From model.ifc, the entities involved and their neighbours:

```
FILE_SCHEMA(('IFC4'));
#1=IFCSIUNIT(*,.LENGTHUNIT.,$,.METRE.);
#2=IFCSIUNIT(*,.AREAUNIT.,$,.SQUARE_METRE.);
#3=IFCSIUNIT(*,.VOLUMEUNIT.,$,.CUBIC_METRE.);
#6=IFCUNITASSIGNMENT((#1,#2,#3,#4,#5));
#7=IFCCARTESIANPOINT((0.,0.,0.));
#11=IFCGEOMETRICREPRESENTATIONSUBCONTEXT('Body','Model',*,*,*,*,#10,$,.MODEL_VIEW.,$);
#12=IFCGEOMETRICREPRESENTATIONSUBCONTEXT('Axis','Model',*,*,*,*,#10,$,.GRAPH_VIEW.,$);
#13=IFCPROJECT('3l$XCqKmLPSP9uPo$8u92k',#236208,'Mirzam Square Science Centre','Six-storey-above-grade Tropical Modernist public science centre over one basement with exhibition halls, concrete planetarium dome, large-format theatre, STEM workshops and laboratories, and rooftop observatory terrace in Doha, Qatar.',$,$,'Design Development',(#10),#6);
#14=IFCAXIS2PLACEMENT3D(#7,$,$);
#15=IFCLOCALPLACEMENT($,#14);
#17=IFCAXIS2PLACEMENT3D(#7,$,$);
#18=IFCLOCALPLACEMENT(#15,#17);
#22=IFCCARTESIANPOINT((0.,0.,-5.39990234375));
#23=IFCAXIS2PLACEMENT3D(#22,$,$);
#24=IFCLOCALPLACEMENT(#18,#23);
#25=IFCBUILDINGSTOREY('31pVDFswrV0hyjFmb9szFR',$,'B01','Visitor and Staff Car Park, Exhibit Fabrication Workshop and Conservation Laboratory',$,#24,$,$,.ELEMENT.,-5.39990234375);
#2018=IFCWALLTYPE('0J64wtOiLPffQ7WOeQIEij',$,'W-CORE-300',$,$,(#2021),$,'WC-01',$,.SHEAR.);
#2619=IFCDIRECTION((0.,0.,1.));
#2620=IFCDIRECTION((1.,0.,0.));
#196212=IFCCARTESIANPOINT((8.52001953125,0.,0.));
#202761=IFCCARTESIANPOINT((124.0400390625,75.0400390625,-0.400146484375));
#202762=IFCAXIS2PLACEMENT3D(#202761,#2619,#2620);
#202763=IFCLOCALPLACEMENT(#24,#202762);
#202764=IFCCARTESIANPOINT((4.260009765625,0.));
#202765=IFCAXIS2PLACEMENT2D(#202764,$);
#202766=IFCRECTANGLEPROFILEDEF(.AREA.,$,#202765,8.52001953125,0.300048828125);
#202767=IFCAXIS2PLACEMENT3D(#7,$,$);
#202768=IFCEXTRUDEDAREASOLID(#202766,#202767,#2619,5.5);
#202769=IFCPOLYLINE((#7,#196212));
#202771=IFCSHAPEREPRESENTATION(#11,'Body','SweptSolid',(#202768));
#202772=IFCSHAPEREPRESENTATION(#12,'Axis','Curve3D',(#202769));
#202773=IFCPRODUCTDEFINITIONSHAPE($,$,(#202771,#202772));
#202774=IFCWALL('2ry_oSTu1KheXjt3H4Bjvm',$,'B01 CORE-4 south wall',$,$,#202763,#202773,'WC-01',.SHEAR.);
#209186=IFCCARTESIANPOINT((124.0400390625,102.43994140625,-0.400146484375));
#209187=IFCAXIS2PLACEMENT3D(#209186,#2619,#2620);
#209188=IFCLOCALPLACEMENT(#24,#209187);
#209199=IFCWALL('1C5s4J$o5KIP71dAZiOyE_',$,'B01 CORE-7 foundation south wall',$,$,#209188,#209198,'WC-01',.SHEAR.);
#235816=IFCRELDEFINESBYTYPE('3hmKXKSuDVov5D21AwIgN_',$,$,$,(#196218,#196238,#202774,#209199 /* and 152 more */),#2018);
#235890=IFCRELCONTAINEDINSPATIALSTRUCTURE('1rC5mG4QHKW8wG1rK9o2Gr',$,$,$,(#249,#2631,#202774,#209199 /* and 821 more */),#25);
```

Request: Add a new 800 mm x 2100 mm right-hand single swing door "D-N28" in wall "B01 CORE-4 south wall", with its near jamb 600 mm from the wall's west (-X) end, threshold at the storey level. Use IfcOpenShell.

```python
import numpy as np
import ifcopenshell
import ifcopenshell.api.feature
import ifcopenshell.api.geometry
import ifcopenshell.api.root
import ifcopenshell.api.spatial
import ifcopenshell.geom
import ifcopenshell.util.element
import ifcopenshell.util.placement
import ifcopenshell.util.representation
import ifcopenshell.util.shape
import ifcopenshell.util.unit

model = ifcopenshell.open("model.ifc")
unit_scale = ifcopenshell.util.unit.calculate_unit_scale(model)
settings = ifcopenshell.geom.settings()


def volume(element):
    """Net volume in cubic metres, openings subtracted."""
    shape = ifcopenshell.geom.create_shape(settings, element)
    return ifcopenshell.util.shape.get_volume(shape.geometry)


wall = model.by_guid("2ry_oSTu1KheXjt3H4Bjvm")
storey = ifcopenshell.util.element.get_container(wall, ifc_class="IfcBuildingStorey")
context = ifcopenshell.util.representation.get_context(model, "Model", "Body", "MODEL_VIEW")
before = volume(wall)

width, height, from_end, sill = 0.8, 2.1, 0.6, 0.0  # metres

# The wall runs along its own X axis, and the end named is its -X end.
wall_shape = ifcopenshell.geom.create_shape(settings, wall)
x, y, z = ifcopenshell.util.shape.get_vertices(wall_shape.geometry).T
start = x.min() + from_end
face, thickness = float(y.min()), float(y.max() - y.min())
wall_matrix = ifcopenshell.util.placement.get_local_placement(wall.ObjectPlacement)
level = ifcopenshell.util.placement.get_local_placement(storey.ObjectPlacement)[2, 3]


def in_wall(x, y):
    """Placement at x, y metres in the wall's axes, at sill height."""
    matrix = wall_matrix.copy()
    matrix[:, 3] = wall_matrix @ np.array([x / unit_scale, y / unit_scale, 0.0, 1.0])
    matrix[2, 3] = level + sill / unit_scale
    return matrix


# Opening: a box that overshoots both wall faces by 50 mm.
opening = ifcopenshell.api.root.create_entity(model, ifc_class="IfcOpeningElement", predefined_type="OPENING")
box = ifcopenshell.api.geometry.add_wall_representation(
    model, context=context, length=width, height=height, thickness=thickness + 0.1
)
ifcopenshell.api.geometry.assign_representation(model, product=opening, representation=box)
ifcopenshell.api.geometry.edit_object_placement(model, product=opening, matrix=in_wall(start, face - 0.05), is_si=False)
ifcopenshell.api.feature.add_feature(model, feature=opening, element=wall)

door = ifcopenshell.api.root.create_entity(model, ifc_class="IfcDoor", name="D-N28", predefined_type="DOOR")
door.OverallWidth, door.OverallHeight = width / unit_scale, height / unit_scale
door.OperationType = "SINGLE_SWING_RIGHT"
body = ifcopenshell.api.geometry.add_door_representation(
    model,
    context=context,
    overall_width=door.OverallWidth,
    overall_height=door.OverallHeight,
    operation_type="SINGLE_SWING_RIGHT",
    lining_properties={"LiningDepth": thickness / unit_scale, "ThresholdDepth": thickness / unit_scale},
)
ifcopenshell.api.geometry.assign_representation(model, product=door, representation=body)
ifcopenshell.api.spatial.assign_container(model, products=[door], relating_structure=storey)
ifcopenshell.api.feature.add_filling(model, opening=opening, element=door)

# The lining spans the wall, so the door starts at the wall face.
ifcopenshell.api.geometry.edit_object_placement(model, product=door, matrix=in_wall(start, face), is_si=False)

after = volume(wall)

print(f"wall volume {before:.3f} -> {after:.3f} m3")

model.write("model_rev.ifc")
```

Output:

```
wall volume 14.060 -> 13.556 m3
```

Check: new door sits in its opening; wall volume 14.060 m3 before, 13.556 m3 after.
